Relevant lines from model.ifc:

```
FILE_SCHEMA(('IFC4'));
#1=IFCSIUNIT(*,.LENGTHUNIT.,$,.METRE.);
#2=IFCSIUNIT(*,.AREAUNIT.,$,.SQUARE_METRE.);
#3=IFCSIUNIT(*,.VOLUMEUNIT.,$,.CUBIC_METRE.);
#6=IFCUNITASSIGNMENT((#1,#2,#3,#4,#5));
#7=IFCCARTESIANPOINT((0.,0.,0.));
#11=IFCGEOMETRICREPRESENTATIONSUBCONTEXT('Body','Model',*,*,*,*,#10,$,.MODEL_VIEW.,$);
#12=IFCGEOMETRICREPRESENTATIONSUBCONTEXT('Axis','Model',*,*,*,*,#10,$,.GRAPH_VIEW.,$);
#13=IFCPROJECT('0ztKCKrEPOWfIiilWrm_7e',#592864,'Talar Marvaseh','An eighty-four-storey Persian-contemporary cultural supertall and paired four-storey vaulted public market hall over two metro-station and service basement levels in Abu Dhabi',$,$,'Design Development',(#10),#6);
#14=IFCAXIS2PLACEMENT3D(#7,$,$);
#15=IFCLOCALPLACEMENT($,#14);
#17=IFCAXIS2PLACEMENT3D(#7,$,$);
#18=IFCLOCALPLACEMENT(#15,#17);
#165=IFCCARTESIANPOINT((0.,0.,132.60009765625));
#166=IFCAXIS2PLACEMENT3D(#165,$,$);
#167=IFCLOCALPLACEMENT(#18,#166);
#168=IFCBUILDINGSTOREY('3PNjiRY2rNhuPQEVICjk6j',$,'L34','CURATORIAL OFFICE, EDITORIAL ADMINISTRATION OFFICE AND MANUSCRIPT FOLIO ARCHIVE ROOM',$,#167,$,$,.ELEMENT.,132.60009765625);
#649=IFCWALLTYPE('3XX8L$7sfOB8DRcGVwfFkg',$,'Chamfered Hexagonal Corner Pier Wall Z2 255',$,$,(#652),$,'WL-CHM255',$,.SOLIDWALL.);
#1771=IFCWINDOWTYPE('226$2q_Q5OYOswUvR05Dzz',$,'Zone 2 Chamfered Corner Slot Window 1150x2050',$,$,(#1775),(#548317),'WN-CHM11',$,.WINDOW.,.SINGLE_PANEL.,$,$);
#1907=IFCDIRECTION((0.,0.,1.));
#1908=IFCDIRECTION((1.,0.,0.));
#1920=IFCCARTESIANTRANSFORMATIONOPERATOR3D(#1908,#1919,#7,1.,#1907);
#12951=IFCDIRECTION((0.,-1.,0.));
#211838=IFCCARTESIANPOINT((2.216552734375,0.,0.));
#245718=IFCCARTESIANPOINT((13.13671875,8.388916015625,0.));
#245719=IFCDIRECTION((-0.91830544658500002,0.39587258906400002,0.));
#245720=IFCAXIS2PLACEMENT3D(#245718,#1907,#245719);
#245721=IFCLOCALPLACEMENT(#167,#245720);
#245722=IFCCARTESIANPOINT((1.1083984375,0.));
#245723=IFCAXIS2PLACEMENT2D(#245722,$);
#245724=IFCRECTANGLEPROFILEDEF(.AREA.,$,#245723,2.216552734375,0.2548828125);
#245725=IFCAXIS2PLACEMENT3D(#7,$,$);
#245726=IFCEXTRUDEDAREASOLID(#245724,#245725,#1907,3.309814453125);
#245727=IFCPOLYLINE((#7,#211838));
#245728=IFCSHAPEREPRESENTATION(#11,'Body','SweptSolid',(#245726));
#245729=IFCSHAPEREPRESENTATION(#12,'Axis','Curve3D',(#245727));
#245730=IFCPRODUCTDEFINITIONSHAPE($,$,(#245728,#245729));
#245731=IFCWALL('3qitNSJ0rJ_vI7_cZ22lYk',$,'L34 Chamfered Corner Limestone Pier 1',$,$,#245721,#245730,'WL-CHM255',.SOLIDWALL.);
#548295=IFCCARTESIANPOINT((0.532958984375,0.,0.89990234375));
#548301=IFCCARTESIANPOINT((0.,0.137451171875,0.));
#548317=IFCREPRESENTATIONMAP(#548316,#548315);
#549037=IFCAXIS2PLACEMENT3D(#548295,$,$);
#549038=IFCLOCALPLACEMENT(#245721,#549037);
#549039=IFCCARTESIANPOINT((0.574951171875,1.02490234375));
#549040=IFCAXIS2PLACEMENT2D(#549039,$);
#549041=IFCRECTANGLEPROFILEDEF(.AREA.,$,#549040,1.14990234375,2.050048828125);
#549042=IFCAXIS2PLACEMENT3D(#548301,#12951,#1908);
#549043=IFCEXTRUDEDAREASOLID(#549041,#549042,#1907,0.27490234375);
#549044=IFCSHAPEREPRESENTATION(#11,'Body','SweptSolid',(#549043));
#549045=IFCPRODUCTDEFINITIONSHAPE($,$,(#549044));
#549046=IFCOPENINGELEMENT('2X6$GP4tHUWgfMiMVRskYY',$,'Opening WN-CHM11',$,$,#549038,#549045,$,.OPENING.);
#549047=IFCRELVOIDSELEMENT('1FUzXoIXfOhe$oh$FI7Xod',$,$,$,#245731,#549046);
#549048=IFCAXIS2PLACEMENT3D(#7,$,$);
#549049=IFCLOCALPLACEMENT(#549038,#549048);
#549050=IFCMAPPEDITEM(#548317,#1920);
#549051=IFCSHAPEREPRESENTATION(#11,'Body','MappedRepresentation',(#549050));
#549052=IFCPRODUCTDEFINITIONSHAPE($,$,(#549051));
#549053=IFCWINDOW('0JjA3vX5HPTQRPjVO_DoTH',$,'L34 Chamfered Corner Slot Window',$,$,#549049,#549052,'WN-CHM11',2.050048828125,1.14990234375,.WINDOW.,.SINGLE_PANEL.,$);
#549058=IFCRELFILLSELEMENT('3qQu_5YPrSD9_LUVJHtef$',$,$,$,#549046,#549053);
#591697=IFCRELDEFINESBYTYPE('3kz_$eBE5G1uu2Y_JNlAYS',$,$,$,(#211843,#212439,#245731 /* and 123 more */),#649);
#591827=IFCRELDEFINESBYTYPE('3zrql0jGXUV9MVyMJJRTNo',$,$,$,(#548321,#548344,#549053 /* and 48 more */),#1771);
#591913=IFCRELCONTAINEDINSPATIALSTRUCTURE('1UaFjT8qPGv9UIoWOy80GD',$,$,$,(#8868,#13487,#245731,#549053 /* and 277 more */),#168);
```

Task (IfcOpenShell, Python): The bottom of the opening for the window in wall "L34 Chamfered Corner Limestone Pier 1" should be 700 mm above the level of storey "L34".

```python
import numpy as np
import ifcopenshell
import ifcopenshell.api.geometry
import ifcopenshell.geom
import ifcopenshell.util.element
import ifcopenshell.util.placement
import ifcopenshell.util.shape
import ifcopenshell.util.unit

model = ifcopenshell.open("model.ifc")
unit_scale = ifcopenshell.util.unit.calculate_unit_scale(model)

window = model.by_guid("0JjA3vX5HPTQRPjVO_DoTH")
opening = window.FillsVoids[0].RelatingOpeningElement
storey = ifcopenshell.util.element.get_container(window, ifc_class="IfcBuildingStorey")
level = ifcopenshell.util.placement.get_local_placement(storey.ObjectPlacement)[2, 3]

# The opening's origin need not be at the sill, so measure its lowest point.
shape = ifcopenshell.geom.create_shape(ifcopenshell.geom.settings(), opening)
bottom = ifcopenshell.util.shape.get_shape_bottom_elevation(shape, shape.geometry) / unit_scale
dz = level + 0.7 - bottom

shift = np.array([0.0, 0.0, dz])
# The window is placed relative to its opening, so it follows when the opening moves.
matrix = ifcopenshell.util.placement.get_local_placement(opening.ObjectPlacement)
matrix[:3, 3] += shift
ifcopenshell.api.geometry.edit_object_placement(
    model, product=opening, matrix=matrix, is_si=False, should_transform_children=True
)

print(f"moved by {dz * unit_scale:+.3f} m")

model.write("model-out.ifc")
```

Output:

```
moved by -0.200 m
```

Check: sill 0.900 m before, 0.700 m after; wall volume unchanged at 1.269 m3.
